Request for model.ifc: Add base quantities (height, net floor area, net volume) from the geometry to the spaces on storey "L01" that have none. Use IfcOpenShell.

First a look at what the model holds.

```python
import ifcopenshell
import ifcopenshell.util.element
import ifcopenshell.util.unit

model = ifcopenshell.open("model.ifc")
print(model.schema)
for unit_type in ("LENGTHUNIT", "AREAUNIT", "VOLUMEUNIT"):
    print(unit_type, ifcopenshell.util.unit.calculate_unit_scale(model, unit_type))
storey = next(s for s in model.by_type("IfcBuildingStorey") if s.Name == "L01")
spaces = [e for e in ifcopenshell.util.element.get_decomposition(storey) if e.is_a("IfcSpace")]
for e in sorted(spaces, key=lambda e: e.id()):
    print(e.id(), e.is_a(), e.Name, list(ifcopenshell.util.element.get_psets(e, qtos_only=True)), sep=" | ")
```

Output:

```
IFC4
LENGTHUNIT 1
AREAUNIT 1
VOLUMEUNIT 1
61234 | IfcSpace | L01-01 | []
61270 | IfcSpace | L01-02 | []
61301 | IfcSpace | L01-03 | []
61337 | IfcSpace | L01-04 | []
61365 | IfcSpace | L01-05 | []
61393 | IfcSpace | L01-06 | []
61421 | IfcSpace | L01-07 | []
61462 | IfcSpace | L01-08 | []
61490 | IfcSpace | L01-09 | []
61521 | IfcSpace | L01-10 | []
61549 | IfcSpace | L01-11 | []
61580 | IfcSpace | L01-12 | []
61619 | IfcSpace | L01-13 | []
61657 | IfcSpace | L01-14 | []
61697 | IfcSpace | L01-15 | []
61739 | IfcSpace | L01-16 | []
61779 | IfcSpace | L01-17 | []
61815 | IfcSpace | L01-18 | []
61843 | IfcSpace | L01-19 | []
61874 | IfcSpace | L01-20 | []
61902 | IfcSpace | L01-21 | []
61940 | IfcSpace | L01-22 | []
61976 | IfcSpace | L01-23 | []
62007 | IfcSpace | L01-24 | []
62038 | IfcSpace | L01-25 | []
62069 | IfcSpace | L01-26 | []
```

```python
import ifcopenshell
import ifcopenshell.api.pset
import ifcopenshell.geom
import ifcopenshell.util.element
import ifcopenshell.util.shape
import ifcopenshell.util.unit

model = ifcopenshell.open("model.ifc")
unit_scale = ifcopenshell.util.unit.calculate_unit_scale(model)
area_scale = ifcopenshell.util.unit.calculate_unit_scale(model, "AREAUNIT")
volume_scale = ifcopenshell.util.unit.calculate_unit_scale(model, "VOLUMEUNIT")
settings = ifcopenshell.geom.settings()

storey = next(s for s in model.by_type("IfcBuildingStorey") if s.Name == "L01")
spaces = [e for e in ifcopenshell.util.element.get_decomposition(storey) if e.is_a("IfcSpace")]

for e in sorted(spaces, key=lambda e: e.id()):
    if ifcopenshell.util.element.get_psets(e, qtos_only=True, should_inherit=False):
        continue
    # Geometry comes back in metres, in the element's own axes.
    shape = ifcopenshell.geom.create_shape(settings, e)
    values = {
        "Height": ifcopenshell.util.shape.get_z(shape.geometry) / unit_scale,
        "NetFloorArea": ifcopenshell.util.shape.get_footprint_area(shape.geometry) / area_scale,
        "NetVolume": ifcopenshell.util.shape.get_volume(shape.geometry) / volume_scale,
    }
    qto = ifcopenshell.api.pset.add_qto(model, product=e, name="Qto_SpaceBaseQuantities")
    ifcopenshell.api.pset.edit_qto(model, qto=qto, properties=values)
    print(e.id(), {k: round(v, 3) for k, v in values.items()})

model.write("model_v2.ifc")
```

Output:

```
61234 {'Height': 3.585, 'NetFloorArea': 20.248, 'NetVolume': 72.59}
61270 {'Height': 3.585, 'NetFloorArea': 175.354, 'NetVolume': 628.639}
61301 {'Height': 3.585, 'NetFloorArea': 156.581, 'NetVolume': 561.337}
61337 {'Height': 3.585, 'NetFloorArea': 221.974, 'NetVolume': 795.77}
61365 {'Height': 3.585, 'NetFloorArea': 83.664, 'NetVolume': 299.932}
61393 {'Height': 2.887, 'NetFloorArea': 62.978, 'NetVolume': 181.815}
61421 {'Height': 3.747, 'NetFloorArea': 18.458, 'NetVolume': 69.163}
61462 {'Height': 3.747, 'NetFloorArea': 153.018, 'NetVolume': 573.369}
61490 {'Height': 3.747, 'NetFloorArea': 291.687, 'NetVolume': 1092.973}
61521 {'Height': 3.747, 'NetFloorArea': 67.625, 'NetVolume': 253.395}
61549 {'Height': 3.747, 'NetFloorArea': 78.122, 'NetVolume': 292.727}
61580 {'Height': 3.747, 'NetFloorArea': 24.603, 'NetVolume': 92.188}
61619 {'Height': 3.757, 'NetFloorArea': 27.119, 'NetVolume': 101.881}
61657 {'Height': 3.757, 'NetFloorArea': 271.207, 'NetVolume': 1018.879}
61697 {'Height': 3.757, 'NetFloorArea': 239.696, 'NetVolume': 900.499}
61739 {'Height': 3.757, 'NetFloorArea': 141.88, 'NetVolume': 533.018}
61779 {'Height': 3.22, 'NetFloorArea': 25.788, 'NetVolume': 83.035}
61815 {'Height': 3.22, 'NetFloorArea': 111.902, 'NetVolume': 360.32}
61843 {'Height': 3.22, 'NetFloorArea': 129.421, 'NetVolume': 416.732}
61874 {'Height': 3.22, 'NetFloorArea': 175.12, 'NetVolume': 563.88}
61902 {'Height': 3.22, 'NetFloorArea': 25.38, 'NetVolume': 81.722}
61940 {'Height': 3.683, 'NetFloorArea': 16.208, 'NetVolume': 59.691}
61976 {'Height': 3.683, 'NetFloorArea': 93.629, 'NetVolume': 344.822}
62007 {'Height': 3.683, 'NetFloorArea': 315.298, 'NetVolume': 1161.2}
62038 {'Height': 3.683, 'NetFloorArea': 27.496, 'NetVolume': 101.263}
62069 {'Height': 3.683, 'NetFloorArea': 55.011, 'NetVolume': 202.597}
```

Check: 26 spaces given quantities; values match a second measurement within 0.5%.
